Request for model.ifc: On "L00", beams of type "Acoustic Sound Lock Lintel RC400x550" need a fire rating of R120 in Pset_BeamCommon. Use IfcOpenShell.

First a look at what the model holds.

```python
import ifcopenshell
import ifcopenshell.util.element

model = ifcopenshell.open("model.ifc")
print(model.schema)
storey = next(s for s in model.by_type("IfcBuildingStorey") if s.Name == "L00")
beams = [e for e in ifcopenshell.util.element.get_decomposition(storey) if e.is_a("IfcBeam")]
seen = {}
for e in beams:
    element_type = ifcopenshell.util.element.get_type(e)
    key = (element_type.Name if element_type != e and element_type else None, ifcopenshell.util.element.get_pset(e, "Pset_BeamCommon", "FireRating"))
    seen[key] = seen.get(key, 0) + 1
for (name, value), count in sorted(seen.items(), key=str):
    print(count, "x", name, "|", value)
```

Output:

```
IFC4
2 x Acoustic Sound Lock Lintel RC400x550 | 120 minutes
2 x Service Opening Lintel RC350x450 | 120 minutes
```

```python
import ifcopenshell
import ifcopenshell.api.pset
import ifcopenshell.util.element

model = ifcopenshell.open("model.ifc")

storey = next(s for s in model.by_type("IfcBuildingStorey") if s.Name == "L00")
beams = [e for e in ifcopenshell.util.element.get_decomposition(storey) if e.is_a("IfcBeam")]

count = 0
for e in beams:
    element_type = ifcopenshell.util.element.get_type(e)
    if element_type in (None, e) or element_type.Name != "Acoustic Sound Lock Lintel RC400x550":
        continue
    # add_pset returns the element's existing set when there is one.
    pset = ifcopenshell.api.pset.add_pset(model, product=e, name="Pset_BeamCommon")
    ifcopenshell.api.pset.edit_pset(model, pset=pset, properties={"FireRating": "R120"})
    count += 1

print(count, "beams updated")

model.write("model_edited.ifc")
```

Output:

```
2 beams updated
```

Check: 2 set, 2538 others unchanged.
